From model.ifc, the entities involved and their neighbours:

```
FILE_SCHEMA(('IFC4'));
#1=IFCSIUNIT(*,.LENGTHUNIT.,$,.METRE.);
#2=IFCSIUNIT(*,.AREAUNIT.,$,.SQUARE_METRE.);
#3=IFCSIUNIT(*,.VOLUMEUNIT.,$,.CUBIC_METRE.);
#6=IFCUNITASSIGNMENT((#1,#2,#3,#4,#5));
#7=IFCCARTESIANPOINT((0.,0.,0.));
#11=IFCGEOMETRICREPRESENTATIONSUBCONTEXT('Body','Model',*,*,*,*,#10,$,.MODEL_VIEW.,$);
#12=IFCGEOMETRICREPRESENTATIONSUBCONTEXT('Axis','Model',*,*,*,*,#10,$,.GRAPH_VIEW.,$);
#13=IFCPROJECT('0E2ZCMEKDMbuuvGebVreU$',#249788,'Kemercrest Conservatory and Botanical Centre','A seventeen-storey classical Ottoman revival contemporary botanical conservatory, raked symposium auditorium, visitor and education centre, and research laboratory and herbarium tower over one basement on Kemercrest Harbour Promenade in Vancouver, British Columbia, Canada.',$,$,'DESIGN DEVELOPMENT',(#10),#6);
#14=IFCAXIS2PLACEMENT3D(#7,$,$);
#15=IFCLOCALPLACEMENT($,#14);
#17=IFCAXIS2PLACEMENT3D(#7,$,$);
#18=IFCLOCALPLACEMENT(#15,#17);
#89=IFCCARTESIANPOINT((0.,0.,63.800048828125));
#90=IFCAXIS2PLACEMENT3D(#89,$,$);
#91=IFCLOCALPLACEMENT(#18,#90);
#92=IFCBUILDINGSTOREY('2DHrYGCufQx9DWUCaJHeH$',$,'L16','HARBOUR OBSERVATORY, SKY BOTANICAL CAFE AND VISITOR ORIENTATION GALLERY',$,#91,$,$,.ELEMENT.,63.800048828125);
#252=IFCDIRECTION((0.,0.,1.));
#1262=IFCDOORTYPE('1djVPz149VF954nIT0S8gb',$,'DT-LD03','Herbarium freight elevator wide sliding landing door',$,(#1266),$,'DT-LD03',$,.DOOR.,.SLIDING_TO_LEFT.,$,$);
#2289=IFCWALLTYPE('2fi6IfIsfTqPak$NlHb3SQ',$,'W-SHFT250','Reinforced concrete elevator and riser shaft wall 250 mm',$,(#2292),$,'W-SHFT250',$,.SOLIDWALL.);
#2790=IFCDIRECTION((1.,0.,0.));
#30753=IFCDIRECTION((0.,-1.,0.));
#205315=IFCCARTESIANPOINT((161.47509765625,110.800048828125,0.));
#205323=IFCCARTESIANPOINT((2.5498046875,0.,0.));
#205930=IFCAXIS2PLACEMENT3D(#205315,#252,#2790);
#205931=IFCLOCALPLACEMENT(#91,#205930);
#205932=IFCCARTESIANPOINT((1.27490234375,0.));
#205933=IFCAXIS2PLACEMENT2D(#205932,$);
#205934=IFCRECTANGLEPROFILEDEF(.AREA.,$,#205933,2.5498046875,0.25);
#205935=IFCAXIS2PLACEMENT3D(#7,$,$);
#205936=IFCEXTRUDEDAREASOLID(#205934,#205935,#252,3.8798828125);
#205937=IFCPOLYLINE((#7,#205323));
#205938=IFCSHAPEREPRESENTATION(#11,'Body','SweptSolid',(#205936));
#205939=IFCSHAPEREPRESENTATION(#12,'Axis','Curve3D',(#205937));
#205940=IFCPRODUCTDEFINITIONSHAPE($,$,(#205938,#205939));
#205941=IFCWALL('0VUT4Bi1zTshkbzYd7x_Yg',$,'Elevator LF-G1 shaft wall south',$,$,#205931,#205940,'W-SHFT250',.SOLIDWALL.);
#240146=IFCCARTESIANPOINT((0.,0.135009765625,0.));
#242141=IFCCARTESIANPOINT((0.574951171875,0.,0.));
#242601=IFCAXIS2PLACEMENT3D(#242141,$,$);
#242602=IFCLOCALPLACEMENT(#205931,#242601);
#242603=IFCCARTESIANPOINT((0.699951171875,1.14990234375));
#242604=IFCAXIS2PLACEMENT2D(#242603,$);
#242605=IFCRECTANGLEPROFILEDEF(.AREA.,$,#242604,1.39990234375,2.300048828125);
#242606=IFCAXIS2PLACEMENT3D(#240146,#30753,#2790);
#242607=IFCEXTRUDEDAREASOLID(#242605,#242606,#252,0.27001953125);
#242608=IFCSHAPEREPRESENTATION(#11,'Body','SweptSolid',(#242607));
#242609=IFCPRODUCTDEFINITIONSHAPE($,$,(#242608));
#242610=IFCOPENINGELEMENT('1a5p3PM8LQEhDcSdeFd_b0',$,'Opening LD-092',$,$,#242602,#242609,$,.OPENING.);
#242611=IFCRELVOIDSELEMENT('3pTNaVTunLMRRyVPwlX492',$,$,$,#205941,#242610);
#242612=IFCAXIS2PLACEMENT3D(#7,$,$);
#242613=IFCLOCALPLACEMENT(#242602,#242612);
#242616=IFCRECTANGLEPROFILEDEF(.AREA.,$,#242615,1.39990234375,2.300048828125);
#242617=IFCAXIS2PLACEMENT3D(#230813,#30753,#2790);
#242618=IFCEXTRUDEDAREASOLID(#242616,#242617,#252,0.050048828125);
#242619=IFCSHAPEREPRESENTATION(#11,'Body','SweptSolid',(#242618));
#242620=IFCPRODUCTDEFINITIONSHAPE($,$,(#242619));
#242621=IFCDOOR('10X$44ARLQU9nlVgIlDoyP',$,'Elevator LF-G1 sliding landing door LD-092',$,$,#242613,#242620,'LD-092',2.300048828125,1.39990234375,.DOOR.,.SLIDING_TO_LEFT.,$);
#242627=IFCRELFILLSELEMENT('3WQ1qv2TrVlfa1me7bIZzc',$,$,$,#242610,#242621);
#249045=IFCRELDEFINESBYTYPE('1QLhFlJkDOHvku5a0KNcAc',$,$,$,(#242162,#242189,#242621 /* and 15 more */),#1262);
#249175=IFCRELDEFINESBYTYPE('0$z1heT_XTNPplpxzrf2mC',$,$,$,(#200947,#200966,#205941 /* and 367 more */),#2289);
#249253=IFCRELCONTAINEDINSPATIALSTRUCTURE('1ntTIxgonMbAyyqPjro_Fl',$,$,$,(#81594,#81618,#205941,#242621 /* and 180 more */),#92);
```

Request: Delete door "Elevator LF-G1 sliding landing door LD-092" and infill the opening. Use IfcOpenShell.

```python
import ifcopenshell
import ifcopenshell.api.feature
import ifcopenshell.api.root
import ifcopenshell.geom
import ifcopenshell.util.shape

model = ifcopenshell.open("model.ifc")
settings = ifcopenshell.geom.settings()


def volume(element):
    """Net volume in cubic metres, openings subtracted."""
    shape = ifcopenshell.geom.create_shape(settings, element)
    return ifcopenshell.util.shape.get_volume(shape.geometry)


door = model.by_guid("10X$44ARLQU9nlVgIlDoyP")
opening = door.FillsVoids[0].RelatingOpeningElement
wall = opening.VoidsElements[0].RelatingBuildingElement
before = volume(wall)

ifcopenshell.api.root.remove_product(model, product=door)
ifcopenshell.api.feature.remove_feature(model, feature=opening)

after = volume(wall)

print(f"wall volume {before:.3f} -> {after:.3f} m3")

model.write("model_v2.ifc")
```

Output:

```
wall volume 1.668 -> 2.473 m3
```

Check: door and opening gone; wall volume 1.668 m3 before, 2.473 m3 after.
